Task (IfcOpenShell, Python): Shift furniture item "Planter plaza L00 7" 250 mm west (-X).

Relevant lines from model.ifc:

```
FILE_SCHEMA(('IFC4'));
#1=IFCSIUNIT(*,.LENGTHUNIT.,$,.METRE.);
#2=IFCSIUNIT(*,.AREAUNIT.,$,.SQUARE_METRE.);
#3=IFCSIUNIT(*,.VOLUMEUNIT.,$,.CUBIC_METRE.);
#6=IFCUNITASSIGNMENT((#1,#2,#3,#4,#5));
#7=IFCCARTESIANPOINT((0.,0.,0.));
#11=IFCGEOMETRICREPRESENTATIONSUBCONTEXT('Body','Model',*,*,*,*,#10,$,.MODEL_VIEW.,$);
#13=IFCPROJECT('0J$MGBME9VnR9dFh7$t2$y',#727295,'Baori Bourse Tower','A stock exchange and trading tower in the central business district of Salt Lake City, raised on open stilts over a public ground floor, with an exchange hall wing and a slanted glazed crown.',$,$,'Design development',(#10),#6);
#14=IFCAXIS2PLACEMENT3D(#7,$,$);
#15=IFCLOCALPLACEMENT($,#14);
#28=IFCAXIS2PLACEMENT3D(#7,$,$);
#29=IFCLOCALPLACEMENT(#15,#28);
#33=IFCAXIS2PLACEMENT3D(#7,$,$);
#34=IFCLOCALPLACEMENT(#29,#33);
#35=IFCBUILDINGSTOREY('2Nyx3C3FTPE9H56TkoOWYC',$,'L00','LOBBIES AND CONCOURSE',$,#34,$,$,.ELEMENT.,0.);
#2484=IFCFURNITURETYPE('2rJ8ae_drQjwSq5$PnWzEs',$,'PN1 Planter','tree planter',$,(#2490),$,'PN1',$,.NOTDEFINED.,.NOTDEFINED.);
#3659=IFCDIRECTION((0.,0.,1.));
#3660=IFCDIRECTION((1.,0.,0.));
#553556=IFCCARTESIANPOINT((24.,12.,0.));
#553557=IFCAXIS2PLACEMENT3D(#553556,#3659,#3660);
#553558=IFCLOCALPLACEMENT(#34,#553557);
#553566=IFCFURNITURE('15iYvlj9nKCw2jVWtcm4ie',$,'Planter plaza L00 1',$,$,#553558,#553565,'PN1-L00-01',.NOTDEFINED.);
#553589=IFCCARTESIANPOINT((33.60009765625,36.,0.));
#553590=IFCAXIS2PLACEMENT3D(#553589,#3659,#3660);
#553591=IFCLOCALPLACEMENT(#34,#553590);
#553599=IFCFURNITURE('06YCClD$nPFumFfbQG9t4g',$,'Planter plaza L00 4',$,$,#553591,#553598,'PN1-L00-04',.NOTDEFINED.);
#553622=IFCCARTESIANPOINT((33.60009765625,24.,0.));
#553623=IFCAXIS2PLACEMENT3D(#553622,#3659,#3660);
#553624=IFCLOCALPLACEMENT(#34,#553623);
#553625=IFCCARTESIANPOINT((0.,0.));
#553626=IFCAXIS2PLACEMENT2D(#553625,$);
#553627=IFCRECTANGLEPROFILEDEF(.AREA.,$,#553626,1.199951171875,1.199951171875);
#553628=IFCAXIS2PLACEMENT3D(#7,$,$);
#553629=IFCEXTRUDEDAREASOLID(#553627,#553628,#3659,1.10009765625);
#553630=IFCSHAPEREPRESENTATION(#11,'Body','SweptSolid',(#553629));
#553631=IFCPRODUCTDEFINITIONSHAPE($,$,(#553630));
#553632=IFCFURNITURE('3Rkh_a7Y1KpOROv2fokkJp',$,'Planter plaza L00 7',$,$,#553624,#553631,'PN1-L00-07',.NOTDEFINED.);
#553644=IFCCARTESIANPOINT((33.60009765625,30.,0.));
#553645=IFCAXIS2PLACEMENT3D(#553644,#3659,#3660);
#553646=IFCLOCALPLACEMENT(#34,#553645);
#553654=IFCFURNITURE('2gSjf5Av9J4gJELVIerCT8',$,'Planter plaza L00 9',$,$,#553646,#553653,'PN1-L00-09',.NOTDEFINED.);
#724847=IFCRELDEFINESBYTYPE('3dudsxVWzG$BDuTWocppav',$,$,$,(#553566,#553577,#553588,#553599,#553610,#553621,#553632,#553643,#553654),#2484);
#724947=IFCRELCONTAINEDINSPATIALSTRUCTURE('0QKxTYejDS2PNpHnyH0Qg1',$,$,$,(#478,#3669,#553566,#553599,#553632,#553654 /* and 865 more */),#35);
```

```python
import ifcopenshell
import ifcopenshell.api.geometry
import ifcopenshell.util.placement
import ifcopenshell.util.unit

model = ifcopenshell.open("model.ifc")
unit_scale = ifcopenshell.util.unit.calculate_unit_scale(model)

item = model.by_guid("3Rkh_a7Y1KpOROv2fokkJp")
matrix = ifcopenshell.util.placement.get_local_placement(item.ObjectPlacement)
matrix[0, 3] -= 0.25 / unit_scale
ifcopenshell.api.geometry.edit_object_placement(model, product=item, matrix=matrix, is_si=False)

print(ifcopenshell.util.placement.get_local_placement(item.ObjectPlacement).round(3) + 0.0)

model.write("model-out.ifc")
```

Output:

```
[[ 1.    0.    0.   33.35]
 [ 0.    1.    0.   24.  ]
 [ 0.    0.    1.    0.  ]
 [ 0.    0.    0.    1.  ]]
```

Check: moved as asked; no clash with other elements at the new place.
